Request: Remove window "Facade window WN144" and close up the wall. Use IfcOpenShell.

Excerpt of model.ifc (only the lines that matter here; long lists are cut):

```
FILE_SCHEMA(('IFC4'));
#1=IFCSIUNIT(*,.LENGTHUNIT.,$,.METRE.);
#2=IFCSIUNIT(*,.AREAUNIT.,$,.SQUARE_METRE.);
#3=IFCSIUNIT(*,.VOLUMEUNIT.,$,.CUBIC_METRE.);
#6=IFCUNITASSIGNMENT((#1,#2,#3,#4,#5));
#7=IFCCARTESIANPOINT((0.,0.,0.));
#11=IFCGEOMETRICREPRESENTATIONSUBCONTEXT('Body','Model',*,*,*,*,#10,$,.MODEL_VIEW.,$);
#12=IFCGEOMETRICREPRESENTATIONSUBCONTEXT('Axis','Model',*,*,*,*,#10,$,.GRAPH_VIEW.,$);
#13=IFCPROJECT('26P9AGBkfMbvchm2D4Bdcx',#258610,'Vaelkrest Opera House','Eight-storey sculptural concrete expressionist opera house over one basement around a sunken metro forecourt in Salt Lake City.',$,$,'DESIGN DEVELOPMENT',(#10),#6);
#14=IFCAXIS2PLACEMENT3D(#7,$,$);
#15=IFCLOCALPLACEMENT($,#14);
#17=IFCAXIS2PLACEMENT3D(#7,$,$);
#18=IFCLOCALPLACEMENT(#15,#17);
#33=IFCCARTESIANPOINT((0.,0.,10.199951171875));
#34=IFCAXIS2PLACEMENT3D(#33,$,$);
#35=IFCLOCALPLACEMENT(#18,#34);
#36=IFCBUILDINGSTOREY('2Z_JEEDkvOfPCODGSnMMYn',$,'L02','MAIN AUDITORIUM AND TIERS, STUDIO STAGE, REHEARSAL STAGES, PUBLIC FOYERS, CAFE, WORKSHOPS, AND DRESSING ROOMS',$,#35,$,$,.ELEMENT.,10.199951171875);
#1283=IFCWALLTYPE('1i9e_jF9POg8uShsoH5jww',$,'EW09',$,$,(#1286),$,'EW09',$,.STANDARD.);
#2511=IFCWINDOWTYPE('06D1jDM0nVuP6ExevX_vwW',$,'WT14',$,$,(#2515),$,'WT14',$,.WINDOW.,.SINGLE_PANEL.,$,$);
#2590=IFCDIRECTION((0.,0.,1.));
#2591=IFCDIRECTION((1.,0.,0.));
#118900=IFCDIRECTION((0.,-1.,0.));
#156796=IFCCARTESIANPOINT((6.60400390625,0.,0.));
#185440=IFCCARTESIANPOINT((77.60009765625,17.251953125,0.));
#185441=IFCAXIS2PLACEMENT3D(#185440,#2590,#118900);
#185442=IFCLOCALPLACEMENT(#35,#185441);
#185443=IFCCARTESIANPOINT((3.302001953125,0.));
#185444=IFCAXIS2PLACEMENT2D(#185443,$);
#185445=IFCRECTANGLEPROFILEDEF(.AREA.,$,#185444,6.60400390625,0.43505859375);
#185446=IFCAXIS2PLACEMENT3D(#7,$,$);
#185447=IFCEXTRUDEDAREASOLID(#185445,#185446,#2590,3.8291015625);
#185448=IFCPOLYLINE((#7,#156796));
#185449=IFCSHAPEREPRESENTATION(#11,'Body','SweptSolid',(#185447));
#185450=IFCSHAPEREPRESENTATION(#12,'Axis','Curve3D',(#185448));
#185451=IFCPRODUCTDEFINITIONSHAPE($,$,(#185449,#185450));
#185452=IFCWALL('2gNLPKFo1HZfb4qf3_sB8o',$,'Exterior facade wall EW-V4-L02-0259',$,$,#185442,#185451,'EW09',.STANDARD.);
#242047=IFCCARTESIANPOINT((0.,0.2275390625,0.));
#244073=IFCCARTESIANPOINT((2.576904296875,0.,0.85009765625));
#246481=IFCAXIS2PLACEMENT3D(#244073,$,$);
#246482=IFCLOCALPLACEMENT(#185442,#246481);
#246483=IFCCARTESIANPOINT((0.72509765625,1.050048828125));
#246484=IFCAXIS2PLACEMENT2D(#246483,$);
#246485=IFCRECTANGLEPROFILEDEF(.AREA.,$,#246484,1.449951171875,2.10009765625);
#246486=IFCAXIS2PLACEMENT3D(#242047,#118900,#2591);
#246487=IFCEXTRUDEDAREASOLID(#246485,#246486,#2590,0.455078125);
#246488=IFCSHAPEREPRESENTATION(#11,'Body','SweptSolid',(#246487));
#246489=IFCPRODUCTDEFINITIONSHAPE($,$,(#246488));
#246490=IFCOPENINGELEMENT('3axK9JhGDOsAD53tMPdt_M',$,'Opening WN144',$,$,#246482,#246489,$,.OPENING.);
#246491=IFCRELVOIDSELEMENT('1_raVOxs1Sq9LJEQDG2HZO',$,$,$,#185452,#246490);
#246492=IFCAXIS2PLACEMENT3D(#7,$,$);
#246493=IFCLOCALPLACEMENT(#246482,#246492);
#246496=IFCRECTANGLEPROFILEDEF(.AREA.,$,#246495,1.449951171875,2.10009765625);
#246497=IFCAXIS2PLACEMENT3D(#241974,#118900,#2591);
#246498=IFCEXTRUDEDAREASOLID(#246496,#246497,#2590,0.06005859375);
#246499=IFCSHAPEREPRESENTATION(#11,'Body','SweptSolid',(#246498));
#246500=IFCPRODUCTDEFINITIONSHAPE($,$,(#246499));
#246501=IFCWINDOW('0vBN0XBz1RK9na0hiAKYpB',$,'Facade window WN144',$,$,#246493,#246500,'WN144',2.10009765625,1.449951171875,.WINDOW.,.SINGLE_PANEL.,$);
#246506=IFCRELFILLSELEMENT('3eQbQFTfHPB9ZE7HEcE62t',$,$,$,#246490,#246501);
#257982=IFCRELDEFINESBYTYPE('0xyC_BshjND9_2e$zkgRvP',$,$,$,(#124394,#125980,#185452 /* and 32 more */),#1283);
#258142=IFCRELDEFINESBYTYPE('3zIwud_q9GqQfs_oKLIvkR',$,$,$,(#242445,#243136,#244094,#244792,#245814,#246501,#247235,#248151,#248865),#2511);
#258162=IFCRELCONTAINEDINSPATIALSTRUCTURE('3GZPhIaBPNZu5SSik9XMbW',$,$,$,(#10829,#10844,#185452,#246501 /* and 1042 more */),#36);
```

```python
import ifcopenshell
import ifcopenshell.api.feature
import ifcopenshell.api.root
import ifcopenshell.geom
import ifcopenshell.util.shape

model = ifcopenshell.open("model.ifc")
settings = ifcopenshell.geom.settings()


def volume(element):
    """Net volume in cubic metres, openings subtracted."""
    shape = ifcopenshell.geom.create_shape(settings, element)
    return ifcopenshell.util.shape.get_volume(shape.geometry)


window = model.by_guid("0vBN0XBz1RK9na0hiAKYpB")
opening = window.FillsVoids[0].RelatingOpeningElement
wall = opening.VoidsElements[0].RelatingBuildingElement
before = volume(wall)

ifcopenshell.api.root.remove_product(model, product=window)
ifcopenshell.api.feature.remove_feature(model, feature=opening)

after = volume(wall)

print(f"wall volume {before:.3f} -> {after:.3f} m3")

model.write("model_updated.ifc")
```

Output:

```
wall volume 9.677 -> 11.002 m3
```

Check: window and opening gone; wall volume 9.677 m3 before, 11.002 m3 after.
